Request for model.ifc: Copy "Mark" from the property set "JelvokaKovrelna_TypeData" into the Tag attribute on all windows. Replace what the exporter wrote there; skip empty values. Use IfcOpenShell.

First a look at what the model holds.

```python
import ifcopenshell
import ifcopenshell.util.element

model = ifcopenshell.open("model.ifc")
print(model.schema)
windows = model.by_type("IfcWindow")
print(len(windows), "windows")
for e in windows[:8]:
    source = ifcopenshell.util.element.get_pset(e, "JelvokaKovrelna_TypeData", "Mark")
    target = e.Tag
    print(e.id(), repr(source), repr(target), sep=" | ")
```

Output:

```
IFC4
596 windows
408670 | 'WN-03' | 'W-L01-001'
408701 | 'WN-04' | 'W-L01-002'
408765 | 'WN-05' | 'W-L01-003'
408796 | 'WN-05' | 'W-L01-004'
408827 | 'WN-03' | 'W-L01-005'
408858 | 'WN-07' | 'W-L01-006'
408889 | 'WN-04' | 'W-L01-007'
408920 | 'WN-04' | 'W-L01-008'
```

```python
import ifcopenshell
import ifcopenshell.util.element

model = ifcopenshell.open("model.ifc")

count = 0
for e in model.by_type("IfcWindow"):
    value = ifcopenshell.util.element.get_pset(e, "JelvokaKovrelna_TypeData", "Mark")
    current = e.Tag
    if not value or not value.strip() or current == value:
        continue
    e.Tag = value
    count += 1

print(count, "windows updated")

model.write("model_edited.ifc")
```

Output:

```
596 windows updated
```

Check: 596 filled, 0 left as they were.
